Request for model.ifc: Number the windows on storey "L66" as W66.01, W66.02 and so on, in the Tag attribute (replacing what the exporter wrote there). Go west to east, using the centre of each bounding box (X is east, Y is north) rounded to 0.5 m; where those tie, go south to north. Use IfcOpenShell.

First a look at what the model holds.

```python
import ifcopenshell
import ifcopenshell.util.element
import ifcopenshell.util.placement

model = ifcopenshell.open("model.ifc")
print(model.schema)
storey = next(s for s in model.by_type("IfcBuildingStorey") if s.Name == "L66")
windows = [e for e in ifcopenshell.util.element.get_decomposition(storey) if e.is_a("IfcWindow")]
for e in sorted(windows, key=lambda e: e.id()):
    origin = ifcopenshell.util.placement.get_local_placement(e.ObjectPlacement)[:3, 3]
    print(e.id(), e.Tag, e.Name, origin.round(2) + 0.0, sep=" | ")
```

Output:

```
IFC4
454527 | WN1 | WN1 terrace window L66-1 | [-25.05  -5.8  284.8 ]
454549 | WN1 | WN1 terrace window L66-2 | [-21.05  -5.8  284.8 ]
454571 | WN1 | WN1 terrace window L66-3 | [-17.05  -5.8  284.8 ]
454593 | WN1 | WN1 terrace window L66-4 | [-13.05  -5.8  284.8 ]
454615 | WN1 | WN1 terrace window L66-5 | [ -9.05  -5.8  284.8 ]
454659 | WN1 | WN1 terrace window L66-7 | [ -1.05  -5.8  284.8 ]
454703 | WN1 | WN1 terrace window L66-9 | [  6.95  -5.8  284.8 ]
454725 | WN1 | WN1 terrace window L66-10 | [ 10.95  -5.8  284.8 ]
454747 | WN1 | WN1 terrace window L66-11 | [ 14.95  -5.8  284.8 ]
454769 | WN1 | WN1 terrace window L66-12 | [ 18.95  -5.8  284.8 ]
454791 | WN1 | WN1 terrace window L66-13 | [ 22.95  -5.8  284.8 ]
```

```python
import ifcopenshell
import ifcopenshell.geom
import ifcopenshell.util.element
import ifcopenshell.util.shape

model = ifcopenshell.open("model.ifc")
settings = ifcopenshell.geom.settings()
settings.set("use-world-coords", True)


def centre(element):
    shape = ifcopenshell.geom.create_shape(settings, element)
    return ifcopenshell.util.shape.get_bbox_centroid(shape.geometry)


storey = next(s for s in model.by_type("IfcBuildingStorey") if s.Name == "L66")
windows = [e for e in ifcopenshell.util.element.get_decomposition(storey) if e.is_a("IfcWindow")]

# Insertion points can sit at a corner or the storey origin, so sort by the geometry (in metres).
centres = {e: centre(e) for e in windows}
windows.sort(key=lambda e: (round(centres[e][0] / 0.5), centres[e][1]))

for i, e in enumerate(windows, start=1):
    number = f"W66.{i:02d}"
    e.Tag = number
    print(e.id(), number)

model.write("model-out.ifc")
```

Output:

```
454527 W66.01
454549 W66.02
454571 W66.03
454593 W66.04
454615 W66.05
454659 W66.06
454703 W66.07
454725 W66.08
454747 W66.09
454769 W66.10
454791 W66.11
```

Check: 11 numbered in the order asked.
